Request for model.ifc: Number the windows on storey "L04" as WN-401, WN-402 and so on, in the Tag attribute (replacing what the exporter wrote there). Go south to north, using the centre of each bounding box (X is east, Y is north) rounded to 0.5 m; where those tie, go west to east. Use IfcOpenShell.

First a look at what the model holds.

```python
import ifcopenshell
import ifcopenshell.util.element
import ifcopenshell.util.placement

model = ifcopenshell.open("model.ifc")
print(model.schema)
storey = next(s for s in model.by_type("IfcBuildingStorey") if s.Name == "L04")
windows = [e for e in ifcopenshell.util.element.get_decomposition(storey) if e.is_a("IfcWindow")]
for e in sorted(windows, key=lambda e: e.id()):
    origin = ifcopenshell.util.placement.get_local_placement(e.ObjectPlacement)[:3, 3]
    print(e.id(), e.Tag, e.Name, origin.round(2) + 0.0, sep=" | ")
```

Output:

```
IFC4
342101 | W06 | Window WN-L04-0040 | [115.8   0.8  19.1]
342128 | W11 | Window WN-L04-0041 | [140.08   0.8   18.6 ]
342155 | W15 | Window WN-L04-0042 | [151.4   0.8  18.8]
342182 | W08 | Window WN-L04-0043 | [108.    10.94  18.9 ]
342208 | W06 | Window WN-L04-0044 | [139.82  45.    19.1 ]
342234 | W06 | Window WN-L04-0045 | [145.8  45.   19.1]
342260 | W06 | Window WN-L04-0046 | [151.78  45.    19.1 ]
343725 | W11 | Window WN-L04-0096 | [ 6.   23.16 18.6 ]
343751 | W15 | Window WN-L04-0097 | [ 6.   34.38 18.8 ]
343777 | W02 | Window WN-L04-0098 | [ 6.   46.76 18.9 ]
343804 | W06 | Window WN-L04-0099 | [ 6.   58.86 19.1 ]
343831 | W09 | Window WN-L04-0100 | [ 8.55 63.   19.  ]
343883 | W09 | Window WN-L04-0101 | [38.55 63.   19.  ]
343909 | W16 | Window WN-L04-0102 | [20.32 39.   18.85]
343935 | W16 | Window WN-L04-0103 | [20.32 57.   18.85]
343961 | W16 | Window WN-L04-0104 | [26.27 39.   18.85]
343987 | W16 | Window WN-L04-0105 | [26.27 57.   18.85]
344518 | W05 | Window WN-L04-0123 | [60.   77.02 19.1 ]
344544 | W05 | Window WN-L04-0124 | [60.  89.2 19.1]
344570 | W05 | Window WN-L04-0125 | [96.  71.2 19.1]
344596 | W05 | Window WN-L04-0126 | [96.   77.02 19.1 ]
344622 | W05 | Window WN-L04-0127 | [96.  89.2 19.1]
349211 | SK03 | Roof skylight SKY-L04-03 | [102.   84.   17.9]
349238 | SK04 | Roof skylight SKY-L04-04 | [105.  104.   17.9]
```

```python
import ifcopenshell
import ifcopenshell.geom
import ifcopenshell.util.element
import ifcopenshell.util.shape

model = ifcopenshell.open("model.ifc")
settings = ifcopenshell.geom.settings()
settings.set("use-world-coords", True)


def centre(element):
    shape = ifcopenshell.geom.create_shape(settings, element)
    return ifcopenshell.util.shape.get_bbox_centroid(shape.geometry)


storey = next(s for s in model.by_type("IfcBuildingStorey") if s.Name == "L04")
windows = [e for e in ifcopenshell.util.element.get_decomposition(storey) if e.is_a("IfcWindow")]

# Insertion points can sit at a corner or the storey origin, so sort by the geometry (in metres).
centres = {e: centre(e) for e in windows}
windows.sort(key=lambda e: (round(centres[e][1] / 0.5), centres[e][0]))

for i, e in enumerate(windows, start=1):
    number = f"WN-4{i:02d}"
    e.Tag = number
    print(e.id(), number)

model.write("model_v2.ifc")
```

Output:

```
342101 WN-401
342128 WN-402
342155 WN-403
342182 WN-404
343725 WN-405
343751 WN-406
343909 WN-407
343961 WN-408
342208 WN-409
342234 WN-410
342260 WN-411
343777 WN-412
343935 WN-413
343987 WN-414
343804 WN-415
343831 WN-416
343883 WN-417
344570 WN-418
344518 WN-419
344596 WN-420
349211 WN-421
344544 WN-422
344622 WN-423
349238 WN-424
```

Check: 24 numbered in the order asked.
